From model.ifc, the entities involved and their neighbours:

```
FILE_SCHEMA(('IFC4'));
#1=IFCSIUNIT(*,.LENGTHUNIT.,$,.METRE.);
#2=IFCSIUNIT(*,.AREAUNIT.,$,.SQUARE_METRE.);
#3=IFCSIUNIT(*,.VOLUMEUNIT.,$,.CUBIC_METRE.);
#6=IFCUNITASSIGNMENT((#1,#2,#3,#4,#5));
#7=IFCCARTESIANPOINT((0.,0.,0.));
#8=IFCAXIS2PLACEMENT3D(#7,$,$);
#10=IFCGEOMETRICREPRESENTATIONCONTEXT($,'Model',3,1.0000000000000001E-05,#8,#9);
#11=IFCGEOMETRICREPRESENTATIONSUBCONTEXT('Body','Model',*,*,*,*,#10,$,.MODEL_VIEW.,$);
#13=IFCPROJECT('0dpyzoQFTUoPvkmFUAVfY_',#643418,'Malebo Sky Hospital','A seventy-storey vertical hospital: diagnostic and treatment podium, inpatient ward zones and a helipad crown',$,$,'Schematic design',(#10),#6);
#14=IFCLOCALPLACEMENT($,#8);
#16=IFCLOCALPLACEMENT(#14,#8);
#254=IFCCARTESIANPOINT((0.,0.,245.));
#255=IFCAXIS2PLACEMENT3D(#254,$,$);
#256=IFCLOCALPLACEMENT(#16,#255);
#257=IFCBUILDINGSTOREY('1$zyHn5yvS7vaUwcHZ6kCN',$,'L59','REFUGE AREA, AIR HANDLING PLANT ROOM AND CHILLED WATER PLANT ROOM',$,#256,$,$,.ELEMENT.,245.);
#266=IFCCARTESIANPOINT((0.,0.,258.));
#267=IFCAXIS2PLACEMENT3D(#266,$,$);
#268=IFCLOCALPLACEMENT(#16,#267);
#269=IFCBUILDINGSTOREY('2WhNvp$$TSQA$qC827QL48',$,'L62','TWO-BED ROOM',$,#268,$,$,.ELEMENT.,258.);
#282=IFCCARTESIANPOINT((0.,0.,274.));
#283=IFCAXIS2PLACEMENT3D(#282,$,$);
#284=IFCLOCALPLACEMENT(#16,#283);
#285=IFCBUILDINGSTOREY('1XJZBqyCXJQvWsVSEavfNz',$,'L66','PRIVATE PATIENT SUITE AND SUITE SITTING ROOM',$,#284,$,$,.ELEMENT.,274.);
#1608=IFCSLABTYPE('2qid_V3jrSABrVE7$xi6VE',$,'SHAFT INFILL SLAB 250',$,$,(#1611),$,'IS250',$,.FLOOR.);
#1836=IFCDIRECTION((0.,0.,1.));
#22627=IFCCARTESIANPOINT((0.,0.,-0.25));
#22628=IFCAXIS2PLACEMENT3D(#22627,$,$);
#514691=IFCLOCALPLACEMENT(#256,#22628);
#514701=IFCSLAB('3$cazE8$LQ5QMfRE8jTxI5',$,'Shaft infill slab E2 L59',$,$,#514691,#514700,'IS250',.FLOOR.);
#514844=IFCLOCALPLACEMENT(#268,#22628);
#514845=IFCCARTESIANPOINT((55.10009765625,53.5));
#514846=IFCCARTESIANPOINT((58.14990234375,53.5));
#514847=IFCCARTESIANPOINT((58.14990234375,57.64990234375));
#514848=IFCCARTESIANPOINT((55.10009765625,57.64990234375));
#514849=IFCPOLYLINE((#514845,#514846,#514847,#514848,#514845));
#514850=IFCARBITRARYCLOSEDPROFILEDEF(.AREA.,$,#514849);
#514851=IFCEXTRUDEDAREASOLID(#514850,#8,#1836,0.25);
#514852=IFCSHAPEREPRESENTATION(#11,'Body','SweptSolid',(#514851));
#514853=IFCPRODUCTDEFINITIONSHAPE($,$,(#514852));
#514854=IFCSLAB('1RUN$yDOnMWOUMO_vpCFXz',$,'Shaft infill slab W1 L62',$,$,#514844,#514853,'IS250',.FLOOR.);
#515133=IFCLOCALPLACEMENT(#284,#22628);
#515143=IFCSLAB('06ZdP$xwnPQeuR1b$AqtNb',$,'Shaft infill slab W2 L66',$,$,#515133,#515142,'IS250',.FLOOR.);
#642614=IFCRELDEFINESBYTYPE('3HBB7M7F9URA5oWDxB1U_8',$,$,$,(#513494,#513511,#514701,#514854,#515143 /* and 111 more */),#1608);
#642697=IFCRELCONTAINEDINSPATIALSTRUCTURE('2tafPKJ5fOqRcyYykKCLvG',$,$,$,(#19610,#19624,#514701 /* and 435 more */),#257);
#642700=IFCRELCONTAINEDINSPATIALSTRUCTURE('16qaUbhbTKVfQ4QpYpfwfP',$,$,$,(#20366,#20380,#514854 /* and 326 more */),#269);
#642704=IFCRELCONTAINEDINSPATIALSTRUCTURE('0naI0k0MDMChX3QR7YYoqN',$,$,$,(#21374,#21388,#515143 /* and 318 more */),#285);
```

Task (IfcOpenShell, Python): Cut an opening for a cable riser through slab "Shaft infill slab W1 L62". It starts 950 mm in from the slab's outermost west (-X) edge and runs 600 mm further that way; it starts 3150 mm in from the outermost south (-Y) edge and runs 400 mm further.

```python
import numpy as np
import ifcopenshell
import ifcopenshell.api.feature
import ifcopenshell.api.geometry
import ifcopenshell.api.root
import ifcopenshell.geom
import ifcopenshell.util.placement
import ifcopenshell.util.representation
import ifcopenshell.util.shape
import ifcopenshell.util.unit

model = ifcopenshell.open("model.ifc")
unit_scale = ifcopenshell.util.unit.calculate_unit_scale(model)
settings = ifcopenshell.geom.settings()


def volume(element):
    """Net volume in cubic metres, openings subtracted."""
    shape = ifcopenshell.geom.create_shape(settings, element)
    return ifcopenshell.util.shape.get_volume(shape.geometry)


slab = model.by_guid("1RUN$yDOnMWOUMO_vpCFXz")
before = volume(slab)

# Extent in the slab's own axes, in metres. The edges named are its -X and -Y sides.
slab_shape = ifcopenshell.geom.create_shape(settings, slab)
vertices = ifcopenshell.util.shape.get_vertices(slab_shape.geometry)
x_min, y_min, bottom = vertices.min(axis=0)
top = vertices[:, 2].max()

opening = ifcopenshell.api.root.create_entity(model, ifc_class="IfcOpeningElement", name="Cable riser opening", predefined_type="OPENING")
context = ifcopenshell.util.representation.get_context(model, "Model", "Body", "MODEL_VIEW")
width, depth = 0.6, 0.4
outline = [(0.0, 0.0), (width, 0.0), (width, depth), (0.0, depth), (0.0, 0.0)]
# Overshoot both faces by 50 mm so the cut is clean.
shape = ifcopenshell.api.geometry.add_slab_representation(
    model, context=context, depth=top - bottom + 0.1, polyline=outline
)
ifcopenshell.api.geometry.assign_representation(model, product=opening, representation=shape)

matrix = ifcopenshell.util.placement.get_local_placement(slab.ObjectPlacement)
matrix[:, 3] = matrix @ np.append(np.array([x_min + 0.95, y_min + 3.15, bottom - 0.05]) / unit_scale, 1.0)
ifcopenshell.api.geometry.edit_object_placement(model, product=opening, matrix=matrix, is_si=False)
ifcopenshell.api.feature.add_feature(model, feature=opening, element=slab)

after = volume(slab)

print(f"slab volume {before:.3f} -> {after:.3f} m3")

model.write("model_updated.ifc")
```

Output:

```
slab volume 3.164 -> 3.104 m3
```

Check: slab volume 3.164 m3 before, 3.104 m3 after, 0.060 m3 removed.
